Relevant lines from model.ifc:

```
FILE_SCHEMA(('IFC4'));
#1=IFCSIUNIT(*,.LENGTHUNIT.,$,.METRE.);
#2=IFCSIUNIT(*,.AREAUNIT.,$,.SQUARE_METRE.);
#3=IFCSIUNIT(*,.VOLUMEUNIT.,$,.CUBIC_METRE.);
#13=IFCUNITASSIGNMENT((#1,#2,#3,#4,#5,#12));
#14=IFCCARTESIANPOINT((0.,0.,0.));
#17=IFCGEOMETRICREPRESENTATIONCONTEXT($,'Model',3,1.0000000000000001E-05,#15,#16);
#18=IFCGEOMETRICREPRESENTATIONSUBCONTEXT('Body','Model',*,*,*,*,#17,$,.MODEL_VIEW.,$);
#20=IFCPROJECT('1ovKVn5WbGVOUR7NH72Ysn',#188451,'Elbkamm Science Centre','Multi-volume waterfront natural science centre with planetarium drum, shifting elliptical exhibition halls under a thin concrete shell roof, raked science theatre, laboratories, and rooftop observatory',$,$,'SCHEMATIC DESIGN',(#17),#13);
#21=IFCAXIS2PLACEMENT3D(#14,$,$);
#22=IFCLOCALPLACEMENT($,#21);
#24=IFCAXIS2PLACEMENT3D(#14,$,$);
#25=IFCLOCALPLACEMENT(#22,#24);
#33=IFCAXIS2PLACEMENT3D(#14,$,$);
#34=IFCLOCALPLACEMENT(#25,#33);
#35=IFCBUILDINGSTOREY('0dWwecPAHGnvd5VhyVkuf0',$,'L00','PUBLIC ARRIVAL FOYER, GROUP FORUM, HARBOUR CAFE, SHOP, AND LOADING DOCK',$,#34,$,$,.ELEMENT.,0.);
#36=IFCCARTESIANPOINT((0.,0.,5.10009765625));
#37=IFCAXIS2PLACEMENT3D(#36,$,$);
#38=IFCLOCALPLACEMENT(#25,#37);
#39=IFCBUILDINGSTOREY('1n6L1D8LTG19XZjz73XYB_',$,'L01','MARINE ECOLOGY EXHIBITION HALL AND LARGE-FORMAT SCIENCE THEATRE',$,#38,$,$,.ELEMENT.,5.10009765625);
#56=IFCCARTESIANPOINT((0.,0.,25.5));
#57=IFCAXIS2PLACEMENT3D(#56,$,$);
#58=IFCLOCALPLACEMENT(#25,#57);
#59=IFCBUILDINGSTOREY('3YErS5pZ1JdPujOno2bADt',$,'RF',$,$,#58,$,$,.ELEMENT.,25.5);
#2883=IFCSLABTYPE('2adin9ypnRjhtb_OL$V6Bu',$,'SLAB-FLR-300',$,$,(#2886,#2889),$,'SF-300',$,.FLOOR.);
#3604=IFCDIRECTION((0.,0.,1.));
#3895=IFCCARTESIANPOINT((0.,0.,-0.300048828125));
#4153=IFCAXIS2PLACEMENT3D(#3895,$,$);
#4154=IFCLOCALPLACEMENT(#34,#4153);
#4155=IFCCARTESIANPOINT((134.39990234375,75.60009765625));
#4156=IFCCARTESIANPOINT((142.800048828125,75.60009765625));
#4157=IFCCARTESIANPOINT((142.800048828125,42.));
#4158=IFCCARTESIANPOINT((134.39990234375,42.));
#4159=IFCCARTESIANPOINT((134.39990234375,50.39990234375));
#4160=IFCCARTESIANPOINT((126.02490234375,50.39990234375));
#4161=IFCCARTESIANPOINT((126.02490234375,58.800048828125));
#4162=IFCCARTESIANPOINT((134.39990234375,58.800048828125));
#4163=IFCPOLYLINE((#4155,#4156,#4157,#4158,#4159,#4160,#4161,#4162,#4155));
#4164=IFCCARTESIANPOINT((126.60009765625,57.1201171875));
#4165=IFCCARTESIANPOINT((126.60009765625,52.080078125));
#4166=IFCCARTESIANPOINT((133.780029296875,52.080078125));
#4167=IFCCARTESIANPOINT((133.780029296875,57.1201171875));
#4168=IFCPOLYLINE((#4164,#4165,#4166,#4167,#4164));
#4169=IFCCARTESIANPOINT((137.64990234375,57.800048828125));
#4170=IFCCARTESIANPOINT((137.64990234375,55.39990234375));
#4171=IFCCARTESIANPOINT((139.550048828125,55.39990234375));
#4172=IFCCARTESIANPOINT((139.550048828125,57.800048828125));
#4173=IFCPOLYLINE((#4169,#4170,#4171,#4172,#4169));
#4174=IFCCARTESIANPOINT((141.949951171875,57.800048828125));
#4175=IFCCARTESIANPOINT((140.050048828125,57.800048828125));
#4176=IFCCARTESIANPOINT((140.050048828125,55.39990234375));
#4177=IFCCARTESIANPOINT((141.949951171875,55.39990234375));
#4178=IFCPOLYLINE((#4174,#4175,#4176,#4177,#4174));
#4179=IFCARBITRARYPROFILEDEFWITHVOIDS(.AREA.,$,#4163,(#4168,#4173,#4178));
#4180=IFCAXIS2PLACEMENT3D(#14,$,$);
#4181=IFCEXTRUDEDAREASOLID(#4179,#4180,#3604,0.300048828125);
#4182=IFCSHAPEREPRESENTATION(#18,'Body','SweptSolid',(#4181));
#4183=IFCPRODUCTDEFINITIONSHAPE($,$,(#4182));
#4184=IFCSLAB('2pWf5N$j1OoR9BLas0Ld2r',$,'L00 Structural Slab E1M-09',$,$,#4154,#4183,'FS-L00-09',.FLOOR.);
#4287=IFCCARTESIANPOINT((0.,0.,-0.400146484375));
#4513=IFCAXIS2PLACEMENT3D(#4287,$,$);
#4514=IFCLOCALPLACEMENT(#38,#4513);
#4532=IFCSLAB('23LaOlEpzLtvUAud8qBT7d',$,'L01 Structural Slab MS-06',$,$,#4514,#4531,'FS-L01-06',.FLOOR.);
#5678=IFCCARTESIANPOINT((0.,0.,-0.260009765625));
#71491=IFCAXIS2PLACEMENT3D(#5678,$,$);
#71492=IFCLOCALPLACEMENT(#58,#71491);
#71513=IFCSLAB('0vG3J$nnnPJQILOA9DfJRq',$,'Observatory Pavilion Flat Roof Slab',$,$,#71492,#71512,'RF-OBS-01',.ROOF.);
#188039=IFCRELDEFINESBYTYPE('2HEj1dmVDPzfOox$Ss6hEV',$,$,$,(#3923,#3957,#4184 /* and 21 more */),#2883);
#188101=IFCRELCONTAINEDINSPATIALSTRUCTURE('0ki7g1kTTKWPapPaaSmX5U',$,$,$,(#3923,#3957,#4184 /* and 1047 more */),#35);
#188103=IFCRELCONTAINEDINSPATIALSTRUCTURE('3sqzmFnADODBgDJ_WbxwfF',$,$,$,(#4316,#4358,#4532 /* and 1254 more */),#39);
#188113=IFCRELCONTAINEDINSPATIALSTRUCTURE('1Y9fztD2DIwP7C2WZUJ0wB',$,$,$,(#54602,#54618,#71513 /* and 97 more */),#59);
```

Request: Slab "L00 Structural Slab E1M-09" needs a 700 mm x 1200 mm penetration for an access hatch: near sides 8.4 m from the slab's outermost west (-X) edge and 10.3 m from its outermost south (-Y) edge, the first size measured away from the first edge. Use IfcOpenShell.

```python
import numpy as np
import ifcopenshell
import ifcopenshell.api.feature
import ifcopenshell.api.geometry
import ifcopenshell.api.root
import ifcopenshell.geom
import ifcopenshell.util.placement
import ifcopenshell.util.representation
import ifcopenshell.util.shape
import ifcopenshell.util.unit

model = ifcopenshell.open("model.ifc")
unit_scale = ifcopenshell.util.unit.calculate_unit_scale(model)
settings = ifcopenshell.geom.settings()


def volume(element):
    """Net volume in cubic metres, openings subtracted."""
    shape = ifcopenshell.geom.create_shape(settings, element)
    return ifcopenshell.util.shape.get_volume(shape.geometry)


slab = model.by_id(4184)
before = volume(slab)

# Extent in the slab's own axes, in metres. The edges named are its -X and -Y sides.
slab_shape = ifcopenshell.geom.create_shape(settings, slab)
vertices = ifcopenshell.util.shape.get_vertices(slab_shape.geometry)
x_min, y_min, bottom = vertices.min(axis=0)
top = vertices[:, 2].max()

opening = ifcopenshell.api.root.create_entity(model, ifc_class="IfcOpeningElement", name="Access hatch opening", predefined_type="OPENING")
context = ifcopenshell.util.representation.get_context(model, "Model", "Body", "MODEL_VIEW")
width, depth = 0.7, 1.2
outline = [(0.0, 0.0), (width, 0.0), (width, depth), (0.0, depth), (0.0, 0.0)]
# Overshoot both faces by 50 mm so the cut is clean.
shape = ifcopenshell.api.geometry.add_slab_representation(
    model, context=context, depth=top - bottom + 0.1, polyline=outline
)
ifcopenshell.api.geometry.assign_representation(model, product=opening, representation=shape)

matrix = ifcopenshell.util.placement.get_local_placement(slab.ObjectPlacement)
matrix[:, 3] = matrix @ np.append(np.array([x_min + 8.4, y_min + 10.3, bottom - 0.05]) / unit_scale, 1.0)
ifcopenshell.api.geometry.edit_object_placement(model, product=opening, matrix=matrix, is_si=False)
ifcopenshell.api.feature.add_feature(model, feature=opening, element=slab)

after = volume(slab)

print(f"slab volume {before:.3f} -> {after:.3f} m3")

model.write("model_edited.ifc")
```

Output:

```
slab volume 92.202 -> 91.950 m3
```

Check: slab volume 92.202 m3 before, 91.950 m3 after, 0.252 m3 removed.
